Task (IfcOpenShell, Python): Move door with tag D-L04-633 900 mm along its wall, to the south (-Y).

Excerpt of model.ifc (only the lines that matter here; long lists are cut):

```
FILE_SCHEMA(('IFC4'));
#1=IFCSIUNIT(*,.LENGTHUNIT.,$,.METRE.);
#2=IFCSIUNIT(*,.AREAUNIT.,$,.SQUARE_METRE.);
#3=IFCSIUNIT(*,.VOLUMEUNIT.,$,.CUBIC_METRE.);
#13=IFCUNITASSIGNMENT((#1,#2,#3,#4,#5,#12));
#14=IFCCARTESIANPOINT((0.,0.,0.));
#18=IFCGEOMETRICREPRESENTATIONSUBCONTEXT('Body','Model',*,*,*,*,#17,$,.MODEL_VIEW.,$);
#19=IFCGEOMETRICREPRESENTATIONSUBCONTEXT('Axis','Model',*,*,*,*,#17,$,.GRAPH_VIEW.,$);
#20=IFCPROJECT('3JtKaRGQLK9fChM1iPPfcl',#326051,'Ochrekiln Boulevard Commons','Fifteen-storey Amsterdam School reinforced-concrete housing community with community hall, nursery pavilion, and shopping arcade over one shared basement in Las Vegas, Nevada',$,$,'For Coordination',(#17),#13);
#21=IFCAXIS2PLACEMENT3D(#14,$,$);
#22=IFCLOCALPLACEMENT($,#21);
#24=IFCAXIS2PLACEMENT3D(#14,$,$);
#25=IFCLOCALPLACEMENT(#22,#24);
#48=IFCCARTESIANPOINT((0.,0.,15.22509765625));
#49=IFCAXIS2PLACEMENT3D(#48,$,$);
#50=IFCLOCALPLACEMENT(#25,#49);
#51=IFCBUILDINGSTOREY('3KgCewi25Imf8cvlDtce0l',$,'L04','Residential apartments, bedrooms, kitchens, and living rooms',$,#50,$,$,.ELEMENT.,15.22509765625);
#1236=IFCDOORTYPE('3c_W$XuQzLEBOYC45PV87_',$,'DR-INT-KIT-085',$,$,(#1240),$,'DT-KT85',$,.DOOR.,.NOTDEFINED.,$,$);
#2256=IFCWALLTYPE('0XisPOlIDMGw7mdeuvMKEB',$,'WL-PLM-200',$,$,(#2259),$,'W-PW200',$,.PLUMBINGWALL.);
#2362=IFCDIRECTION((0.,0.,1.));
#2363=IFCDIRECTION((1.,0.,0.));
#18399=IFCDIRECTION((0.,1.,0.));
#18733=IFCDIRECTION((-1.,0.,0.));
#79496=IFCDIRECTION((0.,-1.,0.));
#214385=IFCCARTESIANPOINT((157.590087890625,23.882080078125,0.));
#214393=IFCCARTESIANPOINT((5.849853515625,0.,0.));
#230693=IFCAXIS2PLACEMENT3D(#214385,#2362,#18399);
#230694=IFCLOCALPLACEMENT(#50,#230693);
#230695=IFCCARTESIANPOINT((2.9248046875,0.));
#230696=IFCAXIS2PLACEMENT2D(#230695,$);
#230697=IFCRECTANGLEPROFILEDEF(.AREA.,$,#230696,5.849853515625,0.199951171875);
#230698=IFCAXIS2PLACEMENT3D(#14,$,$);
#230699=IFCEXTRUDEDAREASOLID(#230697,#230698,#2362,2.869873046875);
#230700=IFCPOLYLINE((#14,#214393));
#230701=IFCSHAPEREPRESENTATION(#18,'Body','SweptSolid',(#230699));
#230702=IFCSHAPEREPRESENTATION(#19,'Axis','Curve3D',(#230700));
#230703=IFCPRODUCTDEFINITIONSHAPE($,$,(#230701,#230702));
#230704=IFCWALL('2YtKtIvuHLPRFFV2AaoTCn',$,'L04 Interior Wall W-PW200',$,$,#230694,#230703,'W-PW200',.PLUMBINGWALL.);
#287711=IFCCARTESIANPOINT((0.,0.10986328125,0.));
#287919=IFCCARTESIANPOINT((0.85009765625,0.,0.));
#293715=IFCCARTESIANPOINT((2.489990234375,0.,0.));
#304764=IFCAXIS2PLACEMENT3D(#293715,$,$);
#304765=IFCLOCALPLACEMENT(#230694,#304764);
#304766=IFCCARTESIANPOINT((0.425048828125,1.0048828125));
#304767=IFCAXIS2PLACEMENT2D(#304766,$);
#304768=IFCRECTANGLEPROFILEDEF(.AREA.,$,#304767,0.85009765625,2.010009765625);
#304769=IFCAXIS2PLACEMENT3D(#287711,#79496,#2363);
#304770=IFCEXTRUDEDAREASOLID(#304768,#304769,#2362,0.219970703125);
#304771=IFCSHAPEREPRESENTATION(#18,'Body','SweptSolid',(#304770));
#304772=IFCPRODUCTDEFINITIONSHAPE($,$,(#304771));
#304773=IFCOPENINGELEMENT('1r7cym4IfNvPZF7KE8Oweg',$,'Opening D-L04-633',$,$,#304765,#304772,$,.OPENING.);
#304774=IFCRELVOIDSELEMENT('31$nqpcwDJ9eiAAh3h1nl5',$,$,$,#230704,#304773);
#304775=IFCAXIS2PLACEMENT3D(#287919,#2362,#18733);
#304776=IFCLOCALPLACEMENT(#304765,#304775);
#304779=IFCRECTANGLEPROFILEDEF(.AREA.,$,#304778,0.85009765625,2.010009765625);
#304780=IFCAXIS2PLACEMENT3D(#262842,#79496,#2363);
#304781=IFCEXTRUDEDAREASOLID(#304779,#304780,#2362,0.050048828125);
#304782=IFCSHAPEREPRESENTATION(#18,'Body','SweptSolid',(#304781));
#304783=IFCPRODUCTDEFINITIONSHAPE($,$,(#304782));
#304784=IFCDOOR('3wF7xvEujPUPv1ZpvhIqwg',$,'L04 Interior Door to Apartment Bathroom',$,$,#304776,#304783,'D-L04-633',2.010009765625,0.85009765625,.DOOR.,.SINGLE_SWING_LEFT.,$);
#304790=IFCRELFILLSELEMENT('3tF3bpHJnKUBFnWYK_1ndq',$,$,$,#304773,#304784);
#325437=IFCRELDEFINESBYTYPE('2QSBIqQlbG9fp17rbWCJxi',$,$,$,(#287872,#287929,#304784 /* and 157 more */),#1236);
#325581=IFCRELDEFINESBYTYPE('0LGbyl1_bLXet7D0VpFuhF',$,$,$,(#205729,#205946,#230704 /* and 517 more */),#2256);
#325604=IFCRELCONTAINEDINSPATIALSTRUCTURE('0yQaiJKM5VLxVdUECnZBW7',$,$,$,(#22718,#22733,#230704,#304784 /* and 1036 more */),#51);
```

```python
import ifcopenshell
import ifcopenshell.api.geometry
import ifcopenshell.util.placement
import ifcopenshell.util.unit

model = ifcopenshell.open("model.ifc")
unit_scale = ifcopenshell.util.unit.calculate_unit_scale(model)

door = model.by_guid("3wF7xvEujPUPv1ZpvhIqwg")
opening = door.FillsVoids[0].RelatingOpeningElement
wall = opening.VoidsElements[0].RelatingBuildingElement

wall_matrix = ifcopenshell.util.placement.get_local_placement(wall.ObjectPlacement)
shift = wall_matrix[:3, 0] * -0.9 / unit_scale
before = ifcopenshell.util.placement.get_local_placement(door.ObjectPlacement)[:3, 3].copy()

# The door is placed relative to its opening, so it follows when the opening moves.
matrix = ifcopenshell.util.placement.get_local_placement(opening.ObjectPlacement)
matrix[:3, 3] += shift
ifcopenshell.api.geometry.edit_object_placement(
    model, product=opening, matrix=matrix, is_si=False, should_transform_children=True
)

after = ifcopenshell.util.placement.get_local_placement(door.ObjectPlacement)[:3, 3]
print("door moved by", (after - before).round(3) + 0.0)

model.write("model-out.ifc")
```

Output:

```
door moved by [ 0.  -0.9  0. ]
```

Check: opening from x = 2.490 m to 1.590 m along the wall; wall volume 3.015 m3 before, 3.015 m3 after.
